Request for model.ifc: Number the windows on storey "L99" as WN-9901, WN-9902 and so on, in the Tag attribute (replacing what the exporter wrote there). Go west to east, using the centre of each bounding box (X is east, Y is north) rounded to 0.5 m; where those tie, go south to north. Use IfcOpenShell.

First a look at what the model holds.

```python
import ifcopenshell
import ifcopenshell.util.element
import ifcopenshell.util.placement

model = ifcopenshell.open("model.ifc")
print(model.schema)
storey = next(s for s in model.by_type("IfcBuildingStorey") if s.Name == "L99")
windows = [e for e in ifcopenshell.util.element.get_decomposition(storey) if e.is_a("IfcWindow")]
for e in sorted(windows, key=lambda e: e.id()):
    origin = ifcopenshell.util.placement.get_local_placement(e.ObjectPlacement)[:3, 3]
    print(e.id(), e.Tag, e.Name, origin.round(2) + 0.0, sep=" | ")
```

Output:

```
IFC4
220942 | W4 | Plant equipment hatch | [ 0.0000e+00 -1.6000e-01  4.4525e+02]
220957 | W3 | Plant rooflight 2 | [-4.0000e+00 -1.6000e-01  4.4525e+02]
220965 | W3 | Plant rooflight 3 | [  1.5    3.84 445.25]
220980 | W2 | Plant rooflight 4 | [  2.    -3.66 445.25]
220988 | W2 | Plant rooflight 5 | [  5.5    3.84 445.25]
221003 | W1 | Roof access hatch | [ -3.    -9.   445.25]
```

```python
import ifcopenshell
import ifcopenshell.geom
import ifcopenshell.util.element
import ifcopenshell.util.shape

model = ifcopenshell.open("model.ifc")
settings = ifcopenshell.geom.settings()
settings.set("use-world-coords", True)


def centre(element):
    shape = ifcopenshell.geom.create_shape(settings, element)
    return ifcopenshell.util.shape.get_bbox_centroid(shape.geometry)


storey = next(s for s in model.by_type("IfcBuildingStorey") if s.Name == "L99")
windows = [e for e in ifcopenshell.util.element.get_decomposition(storey) if e.is_a("IfcWindow")]

# Insertion points can sit at a corner or the storey origin, so sort by the geometry (in metres).
centres = {e: centre(e) for e in windows}
windows.sort(key=lambda e: (round(centres[e][0] / 0.5), centres[e][1]))

for i, e in enumerate(windows, start=1):
    number = f"WN-99{i:02d}"
    e.Tag = number
    print(e.id(), number)

model.write("model_v2.ifc")
```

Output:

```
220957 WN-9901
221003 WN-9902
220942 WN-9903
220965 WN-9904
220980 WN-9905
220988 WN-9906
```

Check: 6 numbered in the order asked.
